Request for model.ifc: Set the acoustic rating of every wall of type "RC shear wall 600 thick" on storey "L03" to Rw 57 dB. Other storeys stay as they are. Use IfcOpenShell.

First a look at what the model holds.

```python
import ifcopenshell
import ifcopenshell.util.element

model = ifcopenshell.open("model.ifc")
print(model.schema)
storey = next(s for s in model.by_type("IfcBuildingStorey") if s.Name == "L03")
walls = [e for e in ifcopenshell.util.element.get_decomposition(storey) if e.is_a("IfcWall")]
seen = {}
for e in walls:
    element_type = ifcopenshell.util.element.get_type(e)
    key = (element_type.Name if element_type != e and element_type else None, ifcopenshell.util.element.get_pset(e, "Pset_WallCommon", "AcousticRating"))
    seen[key] = seen.get(key, 0) + 1
for (name, value), count in sorted(seen.items(), key=str):
    print(count, "x", name, "|", value)
```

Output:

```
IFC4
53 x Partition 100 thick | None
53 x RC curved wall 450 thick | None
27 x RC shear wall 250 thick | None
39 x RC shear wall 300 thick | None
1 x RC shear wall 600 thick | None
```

```python
import ifcopenshell
import ifcopenshell.api.pset
import ifcopenshell.util.element

model = ifcopenshell.open("model.ifc")

storey = next(s for s in model.by_type("IfcBuildingStorey") if s.Name == "L03")
walls = [e for e in ifcopenshell.util.element.get_decomposition(storey) if e.is_a("IfcWall")]

count = 0
for e in walls:
    element_type = ifcopenshell.util.element.get_type(e)
    if element_type in (None, e) or element_type.Name != "RC shear wall 600 thick":
        continue
    # add_pset returns the element's existing set when there is one.
    pset = ifcopenshell.api.pset.add_pset(model, product=e, name="Pset_WallCommon")
    ifcopenshell.api.pset.edit_pset(model, pset=pset, properties={"AcousticRating": "Rw 57 dB"})
    count += 1

print(count, "walls updated")

model.write("model_rev.ifc")
```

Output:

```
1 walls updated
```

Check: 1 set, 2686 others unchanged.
